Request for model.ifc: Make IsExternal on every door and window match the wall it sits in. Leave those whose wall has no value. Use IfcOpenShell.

First a look at what the model holds.

```python
import ifcopenshell
import ifcopenshell.util.element

model = ifcopenshell.open("model.ifc")
print(model.schema)
seen = {}
for e in model.by_type("IfcDoor") + model.by_type("IfcWindow"):
    if not e.FillsVoids:
        continue
    host = e.FillsVoids[0].RelatingOpeningElement.VoidsElements[0].RelatingBuildingElement
    own = ifcopenshell.util.element.get_pset(e, f"Pset_{e.is_a()[3:].removesuffix('StandardCase')}Common", "IsExternal")
    wall = ifcopenshell.util.element.get_pset(host, "Pset_WallCommon", "IsExternal")
    seen[e.is_a(), own, wall] = seen.get((e.is_a(), own, wall), 0) + 1
for (cls, own, wall), count in sorted(seen.items(), key=str):
    print(count, cls, "IsExternal:", own, "| host wall:", wall)
```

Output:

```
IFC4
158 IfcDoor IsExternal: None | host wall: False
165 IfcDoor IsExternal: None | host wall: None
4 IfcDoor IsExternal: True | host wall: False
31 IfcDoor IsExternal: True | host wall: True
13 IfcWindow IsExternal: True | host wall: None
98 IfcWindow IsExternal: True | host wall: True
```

```python
import ifcopenshell
import ifcopenshell.api.pset
import ifcopenshell.util.element

model = ifcopenshell.open("model.ifc")

count = 0
for ifc_class, pset_name in (("IfcDoor", "Pset_DoorCommon"), ("IfcWindow", "Pset_WindowCommon")):
    for e in model.by_type(ifc_class):
        if not e.FillsVoids:
            continue
        host = e.FillsVoids[0].RelatingOpeningElement.VoidsElements[0].RelatingBuildingElement
        external = ifcopenshell.util.element.get_pset(host, "Pset_WallCommon", "IsExternal")
        if external is None or ifcopenshell.util.element.get_pset(e, pset_name, "IsExternal") == external:
            continue
        pset = ifcopenshell.api.pset.add_pset(model, product=e, name=pset_name)
        ifcopenshell.api.pset.edit_pset(model, pset=pset, properties={"IsExternal": external})
        count += 1

print(count, "updated")

model.write("model_v2.ifc")
```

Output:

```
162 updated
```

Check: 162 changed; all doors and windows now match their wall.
